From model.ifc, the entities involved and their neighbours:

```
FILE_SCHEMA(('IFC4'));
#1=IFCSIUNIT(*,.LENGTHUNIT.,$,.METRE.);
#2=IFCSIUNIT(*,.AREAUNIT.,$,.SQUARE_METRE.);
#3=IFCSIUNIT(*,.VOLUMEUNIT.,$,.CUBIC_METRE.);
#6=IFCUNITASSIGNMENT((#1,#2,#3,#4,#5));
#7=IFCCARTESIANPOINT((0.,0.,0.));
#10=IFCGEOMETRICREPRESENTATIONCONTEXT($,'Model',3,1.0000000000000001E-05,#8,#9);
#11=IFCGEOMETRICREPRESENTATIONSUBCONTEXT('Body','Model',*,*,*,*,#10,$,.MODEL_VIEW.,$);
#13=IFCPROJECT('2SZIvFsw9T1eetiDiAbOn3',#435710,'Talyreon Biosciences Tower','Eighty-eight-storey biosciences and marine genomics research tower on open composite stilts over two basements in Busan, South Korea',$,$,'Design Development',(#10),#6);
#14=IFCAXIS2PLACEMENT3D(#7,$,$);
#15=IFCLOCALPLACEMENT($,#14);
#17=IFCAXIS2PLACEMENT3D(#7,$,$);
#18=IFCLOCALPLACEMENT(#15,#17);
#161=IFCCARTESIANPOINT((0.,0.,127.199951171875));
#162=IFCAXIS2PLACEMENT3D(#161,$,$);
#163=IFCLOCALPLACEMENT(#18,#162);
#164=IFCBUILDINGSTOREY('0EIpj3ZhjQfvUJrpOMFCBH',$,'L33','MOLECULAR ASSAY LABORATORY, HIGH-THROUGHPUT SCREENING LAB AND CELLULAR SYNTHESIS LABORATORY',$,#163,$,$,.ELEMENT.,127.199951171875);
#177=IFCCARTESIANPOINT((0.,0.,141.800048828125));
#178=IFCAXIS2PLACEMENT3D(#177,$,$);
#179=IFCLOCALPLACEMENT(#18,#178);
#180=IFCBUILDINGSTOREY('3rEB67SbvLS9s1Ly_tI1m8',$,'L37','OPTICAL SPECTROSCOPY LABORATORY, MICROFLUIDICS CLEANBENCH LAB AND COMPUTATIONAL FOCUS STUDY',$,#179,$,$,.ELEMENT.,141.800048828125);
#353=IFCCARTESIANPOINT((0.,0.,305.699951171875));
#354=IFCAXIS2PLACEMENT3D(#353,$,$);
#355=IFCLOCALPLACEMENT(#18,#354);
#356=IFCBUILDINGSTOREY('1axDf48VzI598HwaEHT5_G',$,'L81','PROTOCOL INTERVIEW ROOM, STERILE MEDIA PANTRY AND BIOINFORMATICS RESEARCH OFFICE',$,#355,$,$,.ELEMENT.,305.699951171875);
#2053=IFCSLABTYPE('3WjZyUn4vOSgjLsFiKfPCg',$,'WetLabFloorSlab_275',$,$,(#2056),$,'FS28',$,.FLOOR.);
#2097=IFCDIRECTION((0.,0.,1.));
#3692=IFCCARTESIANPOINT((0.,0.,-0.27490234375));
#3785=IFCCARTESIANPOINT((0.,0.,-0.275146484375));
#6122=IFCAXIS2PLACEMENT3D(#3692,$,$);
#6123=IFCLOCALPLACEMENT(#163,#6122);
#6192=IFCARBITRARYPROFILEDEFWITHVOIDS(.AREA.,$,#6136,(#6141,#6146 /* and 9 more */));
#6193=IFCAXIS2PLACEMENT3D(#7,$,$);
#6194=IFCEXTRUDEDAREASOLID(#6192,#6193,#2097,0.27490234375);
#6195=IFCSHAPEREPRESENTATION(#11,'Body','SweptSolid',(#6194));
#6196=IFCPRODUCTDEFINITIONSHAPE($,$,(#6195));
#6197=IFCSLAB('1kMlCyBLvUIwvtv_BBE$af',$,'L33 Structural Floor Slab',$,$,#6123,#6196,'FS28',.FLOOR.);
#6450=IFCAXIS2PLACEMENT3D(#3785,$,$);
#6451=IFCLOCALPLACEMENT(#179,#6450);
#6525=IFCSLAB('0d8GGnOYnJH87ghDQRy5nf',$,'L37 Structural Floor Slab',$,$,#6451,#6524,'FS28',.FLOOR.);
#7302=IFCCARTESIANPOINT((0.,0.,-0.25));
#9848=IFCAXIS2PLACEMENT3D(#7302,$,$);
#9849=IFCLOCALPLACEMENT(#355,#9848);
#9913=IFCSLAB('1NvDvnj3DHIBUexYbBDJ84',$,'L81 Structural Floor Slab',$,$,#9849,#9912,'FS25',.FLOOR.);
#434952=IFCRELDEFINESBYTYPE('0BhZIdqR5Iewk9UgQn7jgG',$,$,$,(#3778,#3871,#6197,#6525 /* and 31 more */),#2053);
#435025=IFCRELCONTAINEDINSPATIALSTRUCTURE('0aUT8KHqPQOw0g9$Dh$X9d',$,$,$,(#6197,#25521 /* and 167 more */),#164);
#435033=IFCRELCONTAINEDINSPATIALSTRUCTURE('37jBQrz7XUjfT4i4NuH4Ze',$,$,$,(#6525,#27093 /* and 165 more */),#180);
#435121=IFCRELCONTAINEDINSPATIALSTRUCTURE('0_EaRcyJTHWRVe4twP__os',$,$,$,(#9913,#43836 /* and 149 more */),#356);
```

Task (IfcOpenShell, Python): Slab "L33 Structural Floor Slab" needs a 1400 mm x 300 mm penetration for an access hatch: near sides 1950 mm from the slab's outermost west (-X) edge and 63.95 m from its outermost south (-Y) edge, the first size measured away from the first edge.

```python
import numpy as np
import ifcopenshell
import ifcopenshell.api.feature
import ifcopenshell.api.geometry
import ifcopenshell.api.root
import ifcopenshell.geom
import ifcopenshell.util.placement
import ifcopenshell.util.representation
import ifcopenshell.util.shape
import ifcopenshell.util.unit

model = ifcopenshell.open("model.ifc")
unit_scale = ifcopenshell.util.unit.calculate_unit_scale(model)
settings = ifcopenshell.geom.settings()


def volume(element):
    """Net volume in cubic metres, openings subtracted."""
    shape = ifcopenshell.geom.create_shape(settings, element)
    return ifcopenshell.util.shape.get_volume(shape.geometry)


slab = model.by_guid("1kMlCyBLvUIwvtv_BBE$af")
before = volume(slab)

# Extent in the slab's own axes, in metres. The edges named are its -X and -Y sides.
slab_shape = ifcopenshell.geom.create_shape(settings, slab)
vertices = ifcopenshell.util.shape.get_vertices(slab_shape.geometry)
x_min, y_min, bottom = vertices.min(axis=0)
top = vertices[:, 2].max()

opening = ifcopenshell.api.root.create_entity(model, ifc_class="IfcOpeningElement", name="Access hatch opening", predefined_type="OPENING")
context = ifcopenshell.util.representation.get_context(model, "Model", "Body", "MODEL_VIEW")
width, depth = 1.4, 0.3
outline = [(0.0, 0.0), (width, 0.0), (width, depth), (0.0, depth), (0.0, 0.0)]
# Overshoot both faces by 50 mm so the cut is clean.
shape = ifcopenshell.api.geometry.add_slab_representation(
    model, context=context, depth=top - bottom + 0.1, polyline=outline
)
ifcopenshell.api.geometry.assign_representation(model, product=opening, representation=shape)

matrix = ifcopenshell.util.placement.get_local_placement(slab.ObjectPlacement)
matrix[:, 3] = matrix @ np.append(np.array([x_min + 1.95, y_min + 63.95, bottom - 0.05]) / unit_scale, 1.0)
ifcopenshell.api.geometry.edit_object_placement(model, product=opening, matrix=matrix, is_si=False)
ifcopenshell.api.feature.add_feature(model, feature=opening, element=slab)

after = volume(slab)

print(f"slab volume {before:.3f} -> {after:.3f} m3")

model.write("model-out.ifc")
```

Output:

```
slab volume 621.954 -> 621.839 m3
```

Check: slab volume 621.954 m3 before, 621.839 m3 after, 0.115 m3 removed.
